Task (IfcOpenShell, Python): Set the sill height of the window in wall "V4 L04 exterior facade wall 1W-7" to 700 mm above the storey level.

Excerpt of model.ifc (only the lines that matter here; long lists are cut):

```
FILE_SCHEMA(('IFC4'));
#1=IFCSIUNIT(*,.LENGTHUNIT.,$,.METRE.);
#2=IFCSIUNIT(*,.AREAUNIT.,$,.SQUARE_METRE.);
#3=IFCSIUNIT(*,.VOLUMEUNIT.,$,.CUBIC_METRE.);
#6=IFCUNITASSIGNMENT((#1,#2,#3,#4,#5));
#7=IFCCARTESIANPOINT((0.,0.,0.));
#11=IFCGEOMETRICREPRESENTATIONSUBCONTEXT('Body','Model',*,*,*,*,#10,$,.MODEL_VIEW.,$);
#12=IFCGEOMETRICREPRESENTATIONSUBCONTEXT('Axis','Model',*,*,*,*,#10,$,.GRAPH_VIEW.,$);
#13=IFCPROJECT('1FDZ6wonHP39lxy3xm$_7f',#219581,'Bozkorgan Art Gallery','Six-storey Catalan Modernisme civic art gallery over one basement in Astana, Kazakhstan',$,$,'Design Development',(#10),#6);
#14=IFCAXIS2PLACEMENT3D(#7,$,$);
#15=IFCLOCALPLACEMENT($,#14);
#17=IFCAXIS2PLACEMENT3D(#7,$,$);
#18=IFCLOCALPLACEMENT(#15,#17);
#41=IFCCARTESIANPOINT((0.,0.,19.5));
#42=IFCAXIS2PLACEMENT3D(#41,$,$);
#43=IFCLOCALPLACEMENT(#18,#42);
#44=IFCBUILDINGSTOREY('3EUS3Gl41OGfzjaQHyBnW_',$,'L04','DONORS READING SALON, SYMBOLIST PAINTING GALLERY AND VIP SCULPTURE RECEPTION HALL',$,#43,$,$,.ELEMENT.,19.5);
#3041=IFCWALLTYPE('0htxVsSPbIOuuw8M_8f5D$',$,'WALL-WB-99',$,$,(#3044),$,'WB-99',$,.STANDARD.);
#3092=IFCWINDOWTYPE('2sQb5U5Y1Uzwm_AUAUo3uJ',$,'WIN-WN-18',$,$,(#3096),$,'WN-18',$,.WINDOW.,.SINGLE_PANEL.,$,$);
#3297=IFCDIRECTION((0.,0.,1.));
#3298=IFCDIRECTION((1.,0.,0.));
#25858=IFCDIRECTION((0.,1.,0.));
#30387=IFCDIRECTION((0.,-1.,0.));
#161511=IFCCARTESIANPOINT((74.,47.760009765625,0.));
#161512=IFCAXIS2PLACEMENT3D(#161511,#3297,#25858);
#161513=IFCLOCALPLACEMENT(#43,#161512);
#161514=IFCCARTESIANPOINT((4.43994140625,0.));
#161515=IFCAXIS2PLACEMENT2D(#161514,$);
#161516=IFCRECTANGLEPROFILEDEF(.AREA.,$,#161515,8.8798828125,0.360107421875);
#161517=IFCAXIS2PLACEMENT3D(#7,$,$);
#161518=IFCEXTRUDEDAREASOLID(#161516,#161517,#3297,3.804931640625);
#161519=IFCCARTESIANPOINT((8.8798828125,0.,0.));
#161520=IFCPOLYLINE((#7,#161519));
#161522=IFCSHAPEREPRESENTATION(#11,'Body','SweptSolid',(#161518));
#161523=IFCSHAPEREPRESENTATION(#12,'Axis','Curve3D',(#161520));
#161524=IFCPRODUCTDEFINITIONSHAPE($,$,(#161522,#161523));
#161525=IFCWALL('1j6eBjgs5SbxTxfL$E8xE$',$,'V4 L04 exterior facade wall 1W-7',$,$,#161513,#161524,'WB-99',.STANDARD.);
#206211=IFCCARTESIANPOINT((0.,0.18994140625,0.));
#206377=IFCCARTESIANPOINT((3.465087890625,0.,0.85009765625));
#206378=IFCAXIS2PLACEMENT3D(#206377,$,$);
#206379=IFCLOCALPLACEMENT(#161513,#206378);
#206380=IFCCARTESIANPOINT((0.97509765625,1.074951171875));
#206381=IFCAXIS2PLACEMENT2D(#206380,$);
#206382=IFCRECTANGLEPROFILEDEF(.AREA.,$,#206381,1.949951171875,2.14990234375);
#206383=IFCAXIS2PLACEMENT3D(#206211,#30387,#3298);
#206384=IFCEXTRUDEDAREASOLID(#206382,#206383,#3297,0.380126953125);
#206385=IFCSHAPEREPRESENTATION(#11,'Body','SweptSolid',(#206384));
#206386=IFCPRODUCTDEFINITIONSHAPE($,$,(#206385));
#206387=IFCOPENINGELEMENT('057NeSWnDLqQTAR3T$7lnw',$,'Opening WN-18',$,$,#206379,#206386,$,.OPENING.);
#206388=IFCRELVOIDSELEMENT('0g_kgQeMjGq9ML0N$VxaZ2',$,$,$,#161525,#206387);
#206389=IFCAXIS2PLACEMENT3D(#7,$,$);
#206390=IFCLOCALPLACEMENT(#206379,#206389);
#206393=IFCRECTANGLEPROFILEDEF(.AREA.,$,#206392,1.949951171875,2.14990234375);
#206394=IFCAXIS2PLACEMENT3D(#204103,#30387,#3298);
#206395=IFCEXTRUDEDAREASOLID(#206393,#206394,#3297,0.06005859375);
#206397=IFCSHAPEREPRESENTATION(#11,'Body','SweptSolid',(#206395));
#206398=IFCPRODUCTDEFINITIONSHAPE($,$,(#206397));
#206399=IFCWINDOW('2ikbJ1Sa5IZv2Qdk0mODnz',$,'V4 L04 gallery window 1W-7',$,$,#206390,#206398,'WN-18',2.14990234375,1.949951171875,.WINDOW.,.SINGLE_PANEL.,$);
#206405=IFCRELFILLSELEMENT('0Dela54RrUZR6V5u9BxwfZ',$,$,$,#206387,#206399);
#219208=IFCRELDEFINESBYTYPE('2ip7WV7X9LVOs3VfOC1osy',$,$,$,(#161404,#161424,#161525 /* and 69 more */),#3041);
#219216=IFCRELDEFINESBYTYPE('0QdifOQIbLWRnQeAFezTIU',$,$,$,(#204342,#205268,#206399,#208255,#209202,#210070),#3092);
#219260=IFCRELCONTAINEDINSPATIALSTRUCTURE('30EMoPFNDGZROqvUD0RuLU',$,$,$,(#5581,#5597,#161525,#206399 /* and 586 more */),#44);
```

```python
import numpy as np
import ifcopenshell
import ifcopenshell.api.geometry
import ifcopenshell.geom
import ifcopenshell.util.element
import ifcopenshell.util.placement
import ifcopenshell.util.shape
import ifcopenshell.util.unit

model = ifcopenshell.open("model.ifc")
unit_scale = ifcopenshell.util.unit.calculate_unit_scale(model)

window = model.by_guid("2ikbJ1Sa5IZv2Qdk0mODnz")
opening = window.FillsVoids[0].RelatingOpeningElement
storey = ifcopenshell.util.element.get_container(window, ifc_class="IfcBuildingStorey")
level = ifcopenshell.util.placement.get_local_placement(storey.ObjectPlacement)[2, 3]

# The opening's origin need not be at the sill, so measure its lowest point.
shape = ifcopenshell.geom.create_shape(ifcopenshell.geom.settings(), opening)
bottom = ifcopenshell.util.shape.get_shape_bottom_elevation(shape, shape.geometry) / unit_scale
dz = level + 0.7 - bottom

shift = np.array([0.0, 0.0, dz])
# The window is placed relative to its opening, so it follows when the opening moves.
matrix = ifcopenshell.util.placement.get_local_placement(opening.ObjectPlacement)
matrix[:3, 3] += shift
ifcopenshell.api.geometry.edit_object_placement(
    model, product=opening, matrix=matrix, is_si=False, should_transform_children=True
)

print(f"moved by {dz * unit_scale:+.3f} m")

model.write("model_rev.ifc")
```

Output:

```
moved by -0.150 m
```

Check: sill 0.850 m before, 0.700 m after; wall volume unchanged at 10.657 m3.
